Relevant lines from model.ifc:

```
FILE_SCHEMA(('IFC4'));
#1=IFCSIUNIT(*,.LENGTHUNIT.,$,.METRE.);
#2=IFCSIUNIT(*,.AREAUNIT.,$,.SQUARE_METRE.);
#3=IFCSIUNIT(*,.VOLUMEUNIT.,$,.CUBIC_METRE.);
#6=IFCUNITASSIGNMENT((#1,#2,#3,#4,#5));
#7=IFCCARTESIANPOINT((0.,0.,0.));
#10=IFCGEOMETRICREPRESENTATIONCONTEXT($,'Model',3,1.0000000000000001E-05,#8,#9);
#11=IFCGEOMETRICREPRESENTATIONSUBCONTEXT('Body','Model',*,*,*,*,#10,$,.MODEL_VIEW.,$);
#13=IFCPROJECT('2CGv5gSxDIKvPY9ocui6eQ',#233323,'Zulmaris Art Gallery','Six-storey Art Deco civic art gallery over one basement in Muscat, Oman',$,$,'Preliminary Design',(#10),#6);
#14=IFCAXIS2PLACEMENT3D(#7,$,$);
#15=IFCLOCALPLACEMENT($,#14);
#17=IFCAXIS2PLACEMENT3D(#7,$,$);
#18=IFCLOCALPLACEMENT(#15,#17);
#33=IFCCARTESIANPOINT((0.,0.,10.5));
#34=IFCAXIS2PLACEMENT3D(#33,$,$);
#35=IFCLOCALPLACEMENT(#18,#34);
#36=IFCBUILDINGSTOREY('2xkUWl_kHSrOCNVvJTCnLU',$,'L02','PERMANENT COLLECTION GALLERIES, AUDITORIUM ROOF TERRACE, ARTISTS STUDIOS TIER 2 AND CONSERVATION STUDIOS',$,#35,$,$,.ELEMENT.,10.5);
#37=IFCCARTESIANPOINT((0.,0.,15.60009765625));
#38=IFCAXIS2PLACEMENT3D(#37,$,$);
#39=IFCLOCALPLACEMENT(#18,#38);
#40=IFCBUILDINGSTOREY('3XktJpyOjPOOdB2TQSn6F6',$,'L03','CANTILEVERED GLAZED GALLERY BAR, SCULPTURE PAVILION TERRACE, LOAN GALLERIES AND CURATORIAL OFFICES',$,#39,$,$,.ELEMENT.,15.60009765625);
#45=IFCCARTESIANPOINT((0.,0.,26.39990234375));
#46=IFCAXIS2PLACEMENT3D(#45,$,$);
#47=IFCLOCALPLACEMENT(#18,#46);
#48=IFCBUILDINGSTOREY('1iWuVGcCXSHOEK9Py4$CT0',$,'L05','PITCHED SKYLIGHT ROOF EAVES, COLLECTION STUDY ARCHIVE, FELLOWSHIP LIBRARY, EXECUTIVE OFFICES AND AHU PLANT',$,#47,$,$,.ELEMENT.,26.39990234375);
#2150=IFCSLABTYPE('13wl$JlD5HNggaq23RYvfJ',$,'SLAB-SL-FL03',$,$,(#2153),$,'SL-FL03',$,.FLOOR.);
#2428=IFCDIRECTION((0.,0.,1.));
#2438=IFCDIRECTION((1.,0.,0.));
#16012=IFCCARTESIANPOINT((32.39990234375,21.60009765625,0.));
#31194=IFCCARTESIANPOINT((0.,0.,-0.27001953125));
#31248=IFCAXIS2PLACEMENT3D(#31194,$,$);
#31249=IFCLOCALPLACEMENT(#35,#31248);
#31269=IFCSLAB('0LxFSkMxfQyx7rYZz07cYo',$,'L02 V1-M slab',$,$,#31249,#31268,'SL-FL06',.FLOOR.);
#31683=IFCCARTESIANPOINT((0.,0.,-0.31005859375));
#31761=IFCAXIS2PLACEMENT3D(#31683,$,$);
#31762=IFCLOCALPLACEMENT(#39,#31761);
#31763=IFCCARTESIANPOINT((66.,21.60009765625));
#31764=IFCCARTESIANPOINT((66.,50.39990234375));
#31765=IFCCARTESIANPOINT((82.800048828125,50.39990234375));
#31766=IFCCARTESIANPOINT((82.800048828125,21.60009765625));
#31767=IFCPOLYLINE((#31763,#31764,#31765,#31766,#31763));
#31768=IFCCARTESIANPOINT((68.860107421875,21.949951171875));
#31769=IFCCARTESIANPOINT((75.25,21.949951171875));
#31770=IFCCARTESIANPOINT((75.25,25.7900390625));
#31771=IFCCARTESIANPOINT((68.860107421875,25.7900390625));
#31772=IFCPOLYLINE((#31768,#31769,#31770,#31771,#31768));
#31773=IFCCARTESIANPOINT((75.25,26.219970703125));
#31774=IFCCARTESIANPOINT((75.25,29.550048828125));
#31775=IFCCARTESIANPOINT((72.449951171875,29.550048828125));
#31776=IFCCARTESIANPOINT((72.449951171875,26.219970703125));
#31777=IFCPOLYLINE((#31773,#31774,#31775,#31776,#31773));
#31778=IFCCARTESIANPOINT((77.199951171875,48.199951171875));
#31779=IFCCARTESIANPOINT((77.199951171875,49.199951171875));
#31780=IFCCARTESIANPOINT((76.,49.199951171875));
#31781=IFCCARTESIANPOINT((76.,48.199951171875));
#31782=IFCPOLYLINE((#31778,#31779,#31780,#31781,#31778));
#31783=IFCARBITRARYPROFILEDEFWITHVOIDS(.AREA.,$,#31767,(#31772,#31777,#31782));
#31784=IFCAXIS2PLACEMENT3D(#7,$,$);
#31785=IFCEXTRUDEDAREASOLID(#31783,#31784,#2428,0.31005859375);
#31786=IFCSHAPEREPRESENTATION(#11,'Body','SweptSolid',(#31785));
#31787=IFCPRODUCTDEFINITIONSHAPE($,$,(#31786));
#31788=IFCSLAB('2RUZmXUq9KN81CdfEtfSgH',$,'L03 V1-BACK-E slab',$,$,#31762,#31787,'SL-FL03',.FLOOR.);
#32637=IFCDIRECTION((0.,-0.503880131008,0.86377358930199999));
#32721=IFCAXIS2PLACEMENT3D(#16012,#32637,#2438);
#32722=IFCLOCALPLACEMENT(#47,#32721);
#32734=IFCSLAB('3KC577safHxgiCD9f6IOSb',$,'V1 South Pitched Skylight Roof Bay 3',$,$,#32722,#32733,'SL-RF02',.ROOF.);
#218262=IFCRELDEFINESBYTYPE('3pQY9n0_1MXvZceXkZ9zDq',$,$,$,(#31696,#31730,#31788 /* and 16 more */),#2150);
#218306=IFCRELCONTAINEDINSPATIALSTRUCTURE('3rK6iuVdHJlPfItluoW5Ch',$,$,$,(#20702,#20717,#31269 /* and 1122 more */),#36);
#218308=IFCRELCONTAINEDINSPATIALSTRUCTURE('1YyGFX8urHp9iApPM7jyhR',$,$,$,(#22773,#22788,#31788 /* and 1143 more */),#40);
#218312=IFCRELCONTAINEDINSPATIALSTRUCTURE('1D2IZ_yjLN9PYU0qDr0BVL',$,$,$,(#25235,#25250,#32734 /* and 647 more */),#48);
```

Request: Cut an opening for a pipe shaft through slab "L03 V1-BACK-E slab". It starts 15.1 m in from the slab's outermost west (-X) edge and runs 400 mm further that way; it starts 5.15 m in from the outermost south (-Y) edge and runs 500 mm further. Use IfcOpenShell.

```python
import numpy as np
import ifcopenshell
import ifcopenshell.api.feature
import ifcopenshell.api.geometry
import ifcopenshell.api.root
import ifcopenshell.geom
import ifcopenshell.util.placement
import ifcopenshell.util.representation
import ifcopenshell.util.shape
import ifcopenshell.util.unit

model = ifcopenshell.open("model.ifc")
unit_scale = ifcopenshell.util.unit.calculate_unit_scale(model)
settings = ifcopenshell.geom.settings()


def volume(element):
    """Net volume in cubic metres, openings subtracted."""
    shape = ifcopenshell.geom.create_shape(settings, element)
    return ifcopenshell.util.shape.get_volume(shape.geometry)


slab = model.by_guid("2RUZmXUq9KN81CdfEtfSgH")
before = volume(slab)

# Extent in the slab's own axes, in metres. The edges named are its -X and -Y sides.
slab_shape = ifcopenshell.geom.create_shape(settings, slab)
vertices = ifcopenshell.util.shape.get_vertices(slab_shape.geometry)
x_min, y_min, bottom = vertices.min(axis=0)
top = vertices[:, 2].max()

opening = ifcopenshell.api.root.create_entity(model, ifc_class="IfcOpeningElement", name="Pipe shaft opening", predefined_type="OPENING")
context = ifcopenshell.util.representation.get_context(model, "Model", "Body", "MODEL_VIEW")
width, depth = 0.4, 0.5
outline = [(0.0, 0.0), (width, 0.0), (width, depth), (0.0, depth), (0.0, 0.0)]
# Overshoot both faces by 50 mm so the cut is clean.
shape = ifcopenshell.api.geometry.add_slab_representation(
    model, context=context, depth=top - bottom + 0.1, polyline=outline
)
ifcopenshell.api.geometry.assign_representation(model, product=opening, representation=shape)

matrix = ifcopenshell.util.placement.get_local_placement(slab.ObjectPlacement)
matrix[:, 3] = matrix @ np.append(np.array([x_min + 15.1, y_min + 5.15, bottom - 0.05]) / unit_scale, 1.0)
ifcopenshell.api.geometry.edit_object_placement(model, product=opening, matrix=matrix, is_si=False)
ifcopenshell.api.feature.add_feature(model, feature=opening, element=slab)

after = volume(slab)

print(f"slab volume {before:.3f} -> {after:.3f} m3")

model.write("model_v2.ifc")
```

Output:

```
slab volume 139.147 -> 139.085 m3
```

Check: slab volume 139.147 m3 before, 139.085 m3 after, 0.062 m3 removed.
